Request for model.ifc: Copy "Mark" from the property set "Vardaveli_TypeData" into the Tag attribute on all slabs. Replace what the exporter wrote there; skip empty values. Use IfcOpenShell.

First a look at what the model holds.

```python
import ifcopenshell
import ifcopenshell.util.element

model = ifcopenshell.open("model.ifc")
print(model.schema)
slabs = model.by_type("IfcSlab")
print(len(slabs), "slabs")
for e in slabs[:8]:
    source = ifcopenshell.util.element.get_pset(e, "Vardaveli_TypeData", "Mark")
    target = e.Tag
    print(e.id(), repr(source), repr(target), sep=" | ")
```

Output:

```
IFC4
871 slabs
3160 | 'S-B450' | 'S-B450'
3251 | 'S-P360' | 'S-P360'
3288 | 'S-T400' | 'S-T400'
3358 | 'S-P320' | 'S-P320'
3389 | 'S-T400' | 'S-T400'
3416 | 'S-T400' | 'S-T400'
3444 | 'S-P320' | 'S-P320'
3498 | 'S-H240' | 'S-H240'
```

```python
import ifcopenshell
import ifcopenshell.util.element

model = ifcopenshell.open("model.ifc")

count = 0
for e in model.by_type("IfcSlab"):
    value = ifcopenshell.util.element.get_pset(e, "Vardaveli_TypeData", "Mark")
    current = e.Tag
    if not value or not value.strip() or current == value:
        continue
    e.Tag = value
    count += 1

print(count, "slabs updated")

model.write("model_updated.ifc")
```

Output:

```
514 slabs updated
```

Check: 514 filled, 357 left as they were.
